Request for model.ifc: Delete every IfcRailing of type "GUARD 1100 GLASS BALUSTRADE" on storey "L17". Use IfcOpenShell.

First a look at what the model holds.

```python
import ifcopenshell
import ifcopenshell.util.element

model = ifcopenshell.open("model.ifc")
print(model.schema)
storey = next(s for s in model.by_type("IfcBuildingStorey") if s.Name == "L17")
railings = [e for e in ifcopenshell.util.element.get_decomposition(storey) if e.is_a("IfcRailing")]
seen = {}
for e in railings:
    element_type = ifcopenshell.util.element.get_type(e)
    name = element_type.Name if element_type not in (None, e) else None
    seen[name] = seen.get(name, 0) + 1
for name, count in sorted(seen.items(), key=str):
    print(count, "x", name)
```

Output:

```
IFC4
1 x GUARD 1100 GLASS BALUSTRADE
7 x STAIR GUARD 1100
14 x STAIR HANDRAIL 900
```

```python
import ifcopenshell
import ifcopenshell.api.root
import ifcopenshell.util.element

model = ifcopenshell.open("model.ifc")

storey = next(s for s in model.by_type("IfcBuildingStorey") if s.Name == "L17")
railings = [e for e in ifcopenshell.util.element.get_decomposition(storey) if e.is_a("IfcRailing")]
targets = [e for e in railings if (t := ifcopenshell.util.element.get_type(e)) not in (None, e) and t.Name == "GUARD 1100 GLASS BALUSTRADE"]

for e in targets:
    ifcopenshell.api.root.remove_product(model, product=e)
print(len(targets), "removed")

model.write("model_rev.ifc")
```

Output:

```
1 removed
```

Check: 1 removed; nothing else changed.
